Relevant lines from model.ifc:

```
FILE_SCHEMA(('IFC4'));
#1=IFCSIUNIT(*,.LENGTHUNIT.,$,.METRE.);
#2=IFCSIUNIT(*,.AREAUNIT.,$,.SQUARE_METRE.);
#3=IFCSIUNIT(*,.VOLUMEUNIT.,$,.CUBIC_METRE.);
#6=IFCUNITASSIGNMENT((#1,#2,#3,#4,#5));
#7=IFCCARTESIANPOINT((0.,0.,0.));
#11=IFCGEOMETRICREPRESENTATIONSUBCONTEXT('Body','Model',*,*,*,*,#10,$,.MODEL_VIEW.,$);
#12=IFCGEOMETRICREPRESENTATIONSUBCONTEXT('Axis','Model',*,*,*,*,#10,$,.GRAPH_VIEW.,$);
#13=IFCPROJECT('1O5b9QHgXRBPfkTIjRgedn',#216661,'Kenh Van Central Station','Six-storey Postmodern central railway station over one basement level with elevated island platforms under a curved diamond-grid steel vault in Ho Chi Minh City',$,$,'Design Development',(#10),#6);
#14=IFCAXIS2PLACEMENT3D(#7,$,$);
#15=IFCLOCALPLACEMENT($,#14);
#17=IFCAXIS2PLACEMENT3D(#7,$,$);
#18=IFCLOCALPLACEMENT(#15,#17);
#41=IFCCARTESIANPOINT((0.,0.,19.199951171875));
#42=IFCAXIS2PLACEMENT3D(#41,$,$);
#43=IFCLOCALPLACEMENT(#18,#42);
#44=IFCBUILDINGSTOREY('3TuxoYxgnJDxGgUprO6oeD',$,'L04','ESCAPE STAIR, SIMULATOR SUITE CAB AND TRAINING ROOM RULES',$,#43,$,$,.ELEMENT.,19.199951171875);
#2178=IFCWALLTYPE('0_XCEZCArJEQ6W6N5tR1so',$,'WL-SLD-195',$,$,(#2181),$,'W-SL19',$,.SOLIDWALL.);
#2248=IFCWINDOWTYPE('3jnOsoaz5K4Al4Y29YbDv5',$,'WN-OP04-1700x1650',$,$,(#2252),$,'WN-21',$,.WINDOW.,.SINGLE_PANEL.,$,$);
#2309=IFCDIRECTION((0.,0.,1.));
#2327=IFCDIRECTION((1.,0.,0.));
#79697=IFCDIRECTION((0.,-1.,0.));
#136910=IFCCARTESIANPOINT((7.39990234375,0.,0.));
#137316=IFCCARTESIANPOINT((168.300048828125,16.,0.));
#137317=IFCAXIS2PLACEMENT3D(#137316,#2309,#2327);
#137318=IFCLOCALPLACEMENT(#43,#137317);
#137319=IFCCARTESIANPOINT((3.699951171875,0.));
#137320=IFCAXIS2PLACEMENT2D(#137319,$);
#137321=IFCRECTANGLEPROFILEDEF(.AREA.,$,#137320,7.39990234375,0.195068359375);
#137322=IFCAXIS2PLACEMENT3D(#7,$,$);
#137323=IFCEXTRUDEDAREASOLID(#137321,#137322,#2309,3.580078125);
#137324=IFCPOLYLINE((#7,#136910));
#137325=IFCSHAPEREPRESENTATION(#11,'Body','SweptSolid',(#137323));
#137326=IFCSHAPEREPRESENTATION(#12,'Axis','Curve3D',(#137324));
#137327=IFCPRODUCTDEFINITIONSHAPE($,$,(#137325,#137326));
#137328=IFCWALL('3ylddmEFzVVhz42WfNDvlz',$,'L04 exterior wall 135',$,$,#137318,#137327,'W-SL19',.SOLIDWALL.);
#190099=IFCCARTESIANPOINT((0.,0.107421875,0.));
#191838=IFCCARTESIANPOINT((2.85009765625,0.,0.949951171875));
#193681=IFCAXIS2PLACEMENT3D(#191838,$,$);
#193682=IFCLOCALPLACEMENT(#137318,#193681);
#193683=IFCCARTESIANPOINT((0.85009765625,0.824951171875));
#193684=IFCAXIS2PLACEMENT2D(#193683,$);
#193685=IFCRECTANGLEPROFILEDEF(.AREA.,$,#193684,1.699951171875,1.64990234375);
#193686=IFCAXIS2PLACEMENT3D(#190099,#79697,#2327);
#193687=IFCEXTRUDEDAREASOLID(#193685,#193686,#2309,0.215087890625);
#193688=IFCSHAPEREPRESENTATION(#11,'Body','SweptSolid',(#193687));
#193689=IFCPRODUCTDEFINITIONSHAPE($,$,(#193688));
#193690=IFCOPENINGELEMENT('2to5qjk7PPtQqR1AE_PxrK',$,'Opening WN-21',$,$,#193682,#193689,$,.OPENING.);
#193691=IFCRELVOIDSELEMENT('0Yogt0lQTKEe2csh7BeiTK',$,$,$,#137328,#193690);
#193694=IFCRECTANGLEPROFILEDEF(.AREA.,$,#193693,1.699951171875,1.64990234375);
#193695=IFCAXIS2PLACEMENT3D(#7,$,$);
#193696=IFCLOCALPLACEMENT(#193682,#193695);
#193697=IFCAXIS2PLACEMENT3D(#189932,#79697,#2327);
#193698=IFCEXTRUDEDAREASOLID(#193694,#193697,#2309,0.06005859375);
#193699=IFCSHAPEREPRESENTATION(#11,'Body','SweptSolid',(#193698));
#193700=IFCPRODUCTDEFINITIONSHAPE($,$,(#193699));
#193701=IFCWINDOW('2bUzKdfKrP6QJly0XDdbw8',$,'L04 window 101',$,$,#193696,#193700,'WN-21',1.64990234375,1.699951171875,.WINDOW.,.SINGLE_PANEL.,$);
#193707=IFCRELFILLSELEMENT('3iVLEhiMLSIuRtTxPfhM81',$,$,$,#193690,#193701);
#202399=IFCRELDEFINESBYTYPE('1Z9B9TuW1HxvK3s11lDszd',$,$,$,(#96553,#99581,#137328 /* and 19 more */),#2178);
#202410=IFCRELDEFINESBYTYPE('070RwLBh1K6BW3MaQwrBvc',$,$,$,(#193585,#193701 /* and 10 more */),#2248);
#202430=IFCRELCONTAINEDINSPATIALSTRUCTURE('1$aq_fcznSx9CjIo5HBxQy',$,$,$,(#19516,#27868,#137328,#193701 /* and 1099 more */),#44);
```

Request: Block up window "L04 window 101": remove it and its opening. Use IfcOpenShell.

```python
import ifcopenshell
import ifcopenshell.api.feature
import ifcopenshell.api.root
import ifcopenshell.geom
import ifcopenshell.util.shape

model = ifcopenshell.open("model.ifc")
settings = ifcopenshell.geom.settings()


def volume(element):
    """Net volume in cubic metres, openings subtracted."""
    shape = ifcopenshell.geom.create_shape(settings, element)
    return ifcopenshell.util.shape.get_volume(shape.geometry)


window = model.by_id(193701)
opening = window.FillsVoids[0].RelatingOpeningElement
wall = opening.VoidsElements[0].RelatingBuildingElement
before = volume(wall)

ifcopenshell.api.root.remove_product(model, product=window)
ifcopenshell.api.feature.remove_feature(model, feature=opening)

after = volume(wall)

print(f"wall volume {before:.3f} -> {after:.3f} m3")

model.write("model_v2.ifc")
```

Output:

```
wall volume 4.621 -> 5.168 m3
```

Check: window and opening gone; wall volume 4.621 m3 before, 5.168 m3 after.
